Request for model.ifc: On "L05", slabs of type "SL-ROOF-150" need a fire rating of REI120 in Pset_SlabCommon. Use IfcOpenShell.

First a look at what the model holds.

```python
import ifcopenshell
import ifcopenshell.util.element

model = ifcopenshell.open("model.ifc")
print(model.schema)
storey = next(s for s in model.by_type("IfcBuildingStorey") if s.Name == "L05")
slabs = [e for e in ifcopenshell.util.element.get_decomposition(storey) if e.is_a("IfcSlab")]
seen = {}
for e in slabs:
    element_type = ifcopenshell.util.element.get_type(e)
    key = (element_type.Name if element_type != e and element_type else None, ifcopenshell.util.element.get_pset(e, "Pset_SlabCommon", "FireRating"))
    seen[key] = seen.get(key, 0) + 1
for (name, value), count in sorted(seen.items(), key=str):
    print(count, "x", name, "|", value)
```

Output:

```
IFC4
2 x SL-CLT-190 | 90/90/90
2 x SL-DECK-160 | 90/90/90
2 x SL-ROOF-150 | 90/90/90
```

```python
import ifcopenshell
import ifcopenshell.api.pset
import ifcopenshell.util.element

model = ifcopenshell.open("model.ifc")

storey = next(s for s in model.by_type("IfcBuildingStorey") if s.Name == "L05")
slabs = [e for e in ifcopenshell.util.element.get_decomposition(storey) if e.is_a("IfcSlab")]

count = 0
for e in slabs:
    element_type = ifcopenshell.util.element.get_type(e)
    if element_type in (None, e) or element_type.Name != "SL-ROOF-150":
        continue
    # add_pset returns the element's existing set when there is one.
    pset = ifcopenshell.api.pset.add_pset(model, product=e, name="Pset_SlabCommon")
    ifcopenshell.api.pset.edit_pset(model, pset=pset, properties={"FireRating": "REI120"})
    count += 1

print(count, "slabs updated")

model.write("model_edited.ifc")
```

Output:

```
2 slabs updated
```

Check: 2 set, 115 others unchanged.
